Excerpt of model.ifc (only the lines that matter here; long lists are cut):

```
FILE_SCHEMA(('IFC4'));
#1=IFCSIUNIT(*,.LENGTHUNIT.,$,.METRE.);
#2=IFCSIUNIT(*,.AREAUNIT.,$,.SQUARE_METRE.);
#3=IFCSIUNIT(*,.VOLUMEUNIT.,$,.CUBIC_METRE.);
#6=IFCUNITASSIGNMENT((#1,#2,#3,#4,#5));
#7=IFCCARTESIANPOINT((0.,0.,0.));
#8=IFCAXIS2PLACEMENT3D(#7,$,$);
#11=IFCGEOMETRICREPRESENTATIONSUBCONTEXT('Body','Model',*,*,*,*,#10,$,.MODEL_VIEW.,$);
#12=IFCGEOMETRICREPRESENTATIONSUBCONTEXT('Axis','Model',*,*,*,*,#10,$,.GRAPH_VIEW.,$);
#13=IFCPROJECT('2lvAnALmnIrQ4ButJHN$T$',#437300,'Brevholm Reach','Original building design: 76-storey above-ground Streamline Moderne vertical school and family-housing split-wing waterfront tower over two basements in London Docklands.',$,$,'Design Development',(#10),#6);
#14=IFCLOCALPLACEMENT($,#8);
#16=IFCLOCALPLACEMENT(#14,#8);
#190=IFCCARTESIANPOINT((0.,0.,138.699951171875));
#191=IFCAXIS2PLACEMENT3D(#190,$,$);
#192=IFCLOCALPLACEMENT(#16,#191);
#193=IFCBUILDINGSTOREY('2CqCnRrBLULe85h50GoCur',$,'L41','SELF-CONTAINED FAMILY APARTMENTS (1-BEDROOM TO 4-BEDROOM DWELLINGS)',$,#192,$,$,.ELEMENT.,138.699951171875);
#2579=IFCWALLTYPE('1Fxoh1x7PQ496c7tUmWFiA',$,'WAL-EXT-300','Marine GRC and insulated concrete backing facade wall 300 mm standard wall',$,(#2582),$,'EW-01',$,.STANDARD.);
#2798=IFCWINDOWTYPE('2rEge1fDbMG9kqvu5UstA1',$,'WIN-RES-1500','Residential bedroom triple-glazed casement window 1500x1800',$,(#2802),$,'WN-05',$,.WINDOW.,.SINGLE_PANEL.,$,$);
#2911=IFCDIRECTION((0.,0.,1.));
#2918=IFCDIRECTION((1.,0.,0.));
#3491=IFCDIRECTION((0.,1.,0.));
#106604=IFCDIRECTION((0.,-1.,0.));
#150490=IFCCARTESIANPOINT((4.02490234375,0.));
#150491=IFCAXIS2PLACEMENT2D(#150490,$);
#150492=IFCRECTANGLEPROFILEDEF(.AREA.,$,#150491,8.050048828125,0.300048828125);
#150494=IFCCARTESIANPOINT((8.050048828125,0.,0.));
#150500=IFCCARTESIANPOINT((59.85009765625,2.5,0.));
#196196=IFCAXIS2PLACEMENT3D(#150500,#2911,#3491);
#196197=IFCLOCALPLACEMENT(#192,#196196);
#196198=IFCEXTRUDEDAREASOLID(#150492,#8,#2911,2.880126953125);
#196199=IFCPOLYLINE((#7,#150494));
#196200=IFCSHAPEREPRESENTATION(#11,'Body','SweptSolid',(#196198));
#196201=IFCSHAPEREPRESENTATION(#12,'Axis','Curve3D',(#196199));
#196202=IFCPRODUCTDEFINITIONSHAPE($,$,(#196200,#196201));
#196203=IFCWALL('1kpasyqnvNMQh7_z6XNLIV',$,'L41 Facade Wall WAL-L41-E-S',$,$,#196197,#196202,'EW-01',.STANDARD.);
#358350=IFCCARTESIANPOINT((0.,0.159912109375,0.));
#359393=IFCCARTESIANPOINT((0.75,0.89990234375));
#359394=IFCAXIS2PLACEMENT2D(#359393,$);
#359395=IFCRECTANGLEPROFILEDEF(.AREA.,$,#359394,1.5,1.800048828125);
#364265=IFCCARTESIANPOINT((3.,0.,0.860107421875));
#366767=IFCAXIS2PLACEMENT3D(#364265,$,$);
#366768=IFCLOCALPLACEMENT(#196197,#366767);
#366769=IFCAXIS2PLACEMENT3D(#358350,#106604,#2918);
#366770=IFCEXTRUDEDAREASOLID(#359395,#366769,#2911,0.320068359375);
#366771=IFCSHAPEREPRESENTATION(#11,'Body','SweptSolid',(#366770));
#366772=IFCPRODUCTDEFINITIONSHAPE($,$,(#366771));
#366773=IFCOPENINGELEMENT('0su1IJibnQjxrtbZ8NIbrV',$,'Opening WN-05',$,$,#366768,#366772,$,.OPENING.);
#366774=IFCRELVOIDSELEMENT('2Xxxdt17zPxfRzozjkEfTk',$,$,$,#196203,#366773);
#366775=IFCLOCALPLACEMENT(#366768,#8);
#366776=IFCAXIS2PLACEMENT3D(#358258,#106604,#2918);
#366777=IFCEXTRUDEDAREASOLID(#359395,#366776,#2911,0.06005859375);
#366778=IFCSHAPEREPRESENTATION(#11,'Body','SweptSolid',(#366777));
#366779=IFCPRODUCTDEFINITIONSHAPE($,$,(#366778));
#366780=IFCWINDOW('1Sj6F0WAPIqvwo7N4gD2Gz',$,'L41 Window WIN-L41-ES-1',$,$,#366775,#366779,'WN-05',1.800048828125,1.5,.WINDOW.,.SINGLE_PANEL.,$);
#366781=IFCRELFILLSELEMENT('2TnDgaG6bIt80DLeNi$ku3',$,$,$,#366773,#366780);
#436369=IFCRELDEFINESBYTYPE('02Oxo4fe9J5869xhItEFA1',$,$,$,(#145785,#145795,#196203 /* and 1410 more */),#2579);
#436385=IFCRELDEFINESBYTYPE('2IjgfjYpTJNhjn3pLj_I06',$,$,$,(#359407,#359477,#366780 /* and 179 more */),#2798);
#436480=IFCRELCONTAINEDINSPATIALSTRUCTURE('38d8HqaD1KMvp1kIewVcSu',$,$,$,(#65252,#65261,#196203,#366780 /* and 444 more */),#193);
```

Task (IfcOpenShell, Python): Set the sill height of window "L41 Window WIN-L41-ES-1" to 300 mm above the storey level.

```python
import numpy as np
import ifcopenshell
import ifcopenshell.api.geometry
import ifcopenshell.geom
import ifcopenshell.util.element
import ifcopenshell.util.placement
import ifcopenshell.util.shape
import ifcopenshell.util.unit

model = ifcopenshell.open("model.ifc")
unit_scale = ifcopenshell.util.unit.calculate_unit_scale(model)

window = model.by_guid("1Sj6F0WAPIqvwo7N4gD2Gz")
opening = window.FillsVoids[0].RelatingOpeningElement
storey = ifcopenshell.util.element.get_container(window, ifc_class="IfcBuildingStorey")
level = ifcopenshell.util.placement.get_local_placement(storey.ObjectPlacement)[2, 3]

# The opening's origin need not be at the sill, so measure its lowest point.
shape = ifcopenshell.geom.create_shape(ifcopenshell.geom.settings(), opening)
bottom = ifcopenshell.util.shape.get_shape_bottom_elevation(shape, shape.geometry) / unit_scale
dz = level + 0.3 / unit_scale - bottom

shift = np.array([0.0, 0.0, dz])
# The window is placed relative to its opening, so it follows when the opening moves.
matrix = ifcopenshell.util.placement.get_local_placement(opening.ObjectPlacement)
matrix[:3, 3] += shift
ifcopenshell.api.geometry.edit_object_placement(
    model, product=opening, matrix=matrix, is_si=False, should_transform_children=True
)

print(f"moved by {dz * unit_scale:+.3f} m")

model.write("model_v2.ifc")
```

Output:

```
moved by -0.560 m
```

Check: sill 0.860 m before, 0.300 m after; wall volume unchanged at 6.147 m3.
